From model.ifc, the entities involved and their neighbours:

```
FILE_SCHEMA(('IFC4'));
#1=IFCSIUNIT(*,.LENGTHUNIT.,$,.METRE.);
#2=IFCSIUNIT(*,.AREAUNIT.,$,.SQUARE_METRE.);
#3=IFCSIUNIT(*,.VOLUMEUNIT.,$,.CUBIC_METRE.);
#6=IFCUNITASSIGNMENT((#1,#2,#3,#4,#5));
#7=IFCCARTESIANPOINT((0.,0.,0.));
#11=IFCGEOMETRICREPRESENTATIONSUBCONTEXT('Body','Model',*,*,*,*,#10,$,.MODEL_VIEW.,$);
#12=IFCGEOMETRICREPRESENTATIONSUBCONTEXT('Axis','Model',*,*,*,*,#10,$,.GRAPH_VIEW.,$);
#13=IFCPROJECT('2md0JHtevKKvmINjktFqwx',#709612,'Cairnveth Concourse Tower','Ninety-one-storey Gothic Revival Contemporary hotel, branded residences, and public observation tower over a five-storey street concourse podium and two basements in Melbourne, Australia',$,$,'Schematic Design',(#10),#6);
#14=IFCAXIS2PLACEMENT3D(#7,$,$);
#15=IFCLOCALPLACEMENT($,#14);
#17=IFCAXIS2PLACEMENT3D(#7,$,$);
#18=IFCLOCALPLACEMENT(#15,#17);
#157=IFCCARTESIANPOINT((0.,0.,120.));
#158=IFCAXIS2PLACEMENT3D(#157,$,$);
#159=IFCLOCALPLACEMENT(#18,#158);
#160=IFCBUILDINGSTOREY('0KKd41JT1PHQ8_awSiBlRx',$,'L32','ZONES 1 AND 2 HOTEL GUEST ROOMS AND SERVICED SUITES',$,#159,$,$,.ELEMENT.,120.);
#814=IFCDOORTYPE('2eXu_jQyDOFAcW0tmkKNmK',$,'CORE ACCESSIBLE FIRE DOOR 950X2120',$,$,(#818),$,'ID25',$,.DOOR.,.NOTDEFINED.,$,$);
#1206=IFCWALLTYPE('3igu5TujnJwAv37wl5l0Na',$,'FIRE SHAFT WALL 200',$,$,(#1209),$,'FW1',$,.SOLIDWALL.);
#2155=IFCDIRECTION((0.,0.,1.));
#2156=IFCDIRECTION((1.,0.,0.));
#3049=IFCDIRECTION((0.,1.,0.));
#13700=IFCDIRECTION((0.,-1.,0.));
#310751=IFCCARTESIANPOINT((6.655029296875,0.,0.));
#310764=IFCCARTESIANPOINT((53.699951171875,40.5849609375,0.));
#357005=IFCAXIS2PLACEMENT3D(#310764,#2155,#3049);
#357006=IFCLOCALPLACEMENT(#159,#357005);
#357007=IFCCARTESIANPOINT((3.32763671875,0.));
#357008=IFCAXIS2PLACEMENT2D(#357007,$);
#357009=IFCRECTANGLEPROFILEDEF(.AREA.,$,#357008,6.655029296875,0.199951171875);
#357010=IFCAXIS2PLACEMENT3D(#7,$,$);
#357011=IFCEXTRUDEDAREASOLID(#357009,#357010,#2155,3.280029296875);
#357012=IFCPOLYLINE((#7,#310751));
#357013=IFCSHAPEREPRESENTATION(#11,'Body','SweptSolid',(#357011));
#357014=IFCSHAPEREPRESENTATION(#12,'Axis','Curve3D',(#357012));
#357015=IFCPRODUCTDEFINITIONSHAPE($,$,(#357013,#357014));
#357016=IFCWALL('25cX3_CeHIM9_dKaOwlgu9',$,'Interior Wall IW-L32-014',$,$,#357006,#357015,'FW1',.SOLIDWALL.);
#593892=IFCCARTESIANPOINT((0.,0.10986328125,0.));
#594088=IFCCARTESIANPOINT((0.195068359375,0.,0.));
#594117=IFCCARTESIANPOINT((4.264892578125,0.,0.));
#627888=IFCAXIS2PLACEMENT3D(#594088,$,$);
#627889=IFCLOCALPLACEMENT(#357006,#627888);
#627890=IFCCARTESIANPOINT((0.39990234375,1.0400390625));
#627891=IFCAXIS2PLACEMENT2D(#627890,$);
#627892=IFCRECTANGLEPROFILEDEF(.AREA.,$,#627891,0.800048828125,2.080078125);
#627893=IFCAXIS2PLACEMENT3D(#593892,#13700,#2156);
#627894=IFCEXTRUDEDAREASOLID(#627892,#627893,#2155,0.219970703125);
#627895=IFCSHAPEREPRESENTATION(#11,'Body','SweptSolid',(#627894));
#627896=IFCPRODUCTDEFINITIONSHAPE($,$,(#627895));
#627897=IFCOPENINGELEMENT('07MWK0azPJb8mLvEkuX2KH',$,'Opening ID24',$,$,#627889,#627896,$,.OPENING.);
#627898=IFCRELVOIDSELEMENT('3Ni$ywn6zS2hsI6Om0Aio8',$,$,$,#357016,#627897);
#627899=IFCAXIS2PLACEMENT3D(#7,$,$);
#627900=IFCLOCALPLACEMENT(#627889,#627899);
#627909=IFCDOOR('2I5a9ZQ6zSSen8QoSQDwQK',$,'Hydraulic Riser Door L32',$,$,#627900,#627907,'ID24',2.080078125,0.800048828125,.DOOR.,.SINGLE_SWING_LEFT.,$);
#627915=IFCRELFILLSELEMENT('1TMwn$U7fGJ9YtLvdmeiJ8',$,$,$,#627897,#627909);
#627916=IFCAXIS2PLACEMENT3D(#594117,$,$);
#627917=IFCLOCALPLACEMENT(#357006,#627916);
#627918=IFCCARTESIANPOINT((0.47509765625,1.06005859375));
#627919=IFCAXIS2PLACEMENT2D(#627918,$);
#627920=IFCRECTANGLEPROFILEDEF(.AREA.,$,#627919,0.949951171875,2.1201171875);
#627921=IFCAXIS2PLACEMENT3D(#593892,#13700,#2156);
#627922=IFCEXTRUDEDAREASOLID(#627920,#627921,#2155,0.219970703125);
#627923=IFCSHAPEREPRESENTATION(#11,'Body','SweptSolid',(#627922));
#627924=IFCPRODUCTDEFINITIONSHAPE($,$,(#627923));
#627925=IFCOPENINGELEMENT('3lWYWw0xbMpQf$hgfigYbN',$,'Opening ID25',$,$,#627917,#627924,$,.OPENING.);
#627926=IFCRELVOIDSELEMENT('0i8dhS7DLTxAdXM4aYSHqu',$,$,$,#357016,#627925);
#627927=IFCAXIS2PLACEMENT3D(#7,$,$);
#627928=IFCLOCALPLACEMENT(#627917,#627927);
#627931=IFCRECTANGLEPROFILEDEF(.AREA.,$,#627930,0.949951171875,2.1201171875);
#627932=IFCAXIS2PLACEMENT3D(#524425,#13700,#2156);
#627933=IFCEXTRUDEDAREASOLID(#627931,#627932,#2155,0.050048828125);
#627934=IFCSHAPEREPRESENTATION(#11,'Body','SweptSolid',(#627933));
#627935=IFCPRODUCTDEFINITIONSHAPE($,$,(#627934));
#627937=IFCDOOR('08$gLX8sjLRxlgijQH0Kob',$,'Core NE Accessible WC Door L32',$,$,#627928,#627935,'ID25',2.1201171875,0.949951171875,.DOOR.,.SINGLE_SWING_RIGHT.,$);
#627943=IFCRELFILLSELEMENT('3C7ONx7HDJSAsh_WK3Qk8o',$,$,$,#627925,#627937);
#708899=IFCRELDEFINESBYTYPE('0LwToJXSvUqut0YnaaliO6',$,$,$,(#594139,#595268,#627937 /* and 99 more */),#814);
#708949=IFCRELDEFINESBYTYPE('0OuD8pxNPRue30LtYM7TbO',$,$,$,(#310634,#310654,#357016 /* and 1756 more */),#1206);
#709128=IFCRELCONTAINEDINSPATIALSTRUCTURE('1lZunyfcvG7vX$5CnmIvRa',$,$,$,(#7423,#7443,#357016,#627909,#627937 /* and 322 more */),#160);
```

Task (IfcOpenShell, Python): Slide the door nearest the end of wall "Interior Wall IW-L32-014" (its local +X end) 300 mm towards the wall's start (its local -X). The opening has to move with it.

```python
import ifcopenshell
import ifcopenshell.api.geometry
import ifcopenshell.util.placement
import ifcopenshell.util.unit

model = ifcopenshell.open("model.ifc")
unit_scale = ifcopenshell.util.unit.calculate_unit_scale(model)

door = model.by_guid("08$gLX8sjLRxlgijQH0Kob")
opening = door.FillsVoids[0].RelatingOpeningElement
wall = opening.VoidsElements[0].RelatingBuildingElement

wall_matrix = ifcopenshell.util.placement.get_local_placement(wall.ObjectPlacement)
shift = wall_matrix[:3, 0] * -0.3 / unit_scale
before = ifcopenshell.util.placement.get_local_placement(door.ObjectPlacement)[:3, 3].copy()

# The door is placed relative to its opening, so it follows when the opening moves.
matrix = ifcopenshell.util.placement.get_local_placement(opening.ObjectPlacement)
matrix[:3, 3] += shift
ifcopenshell.api.geometry.edit_object_placement(
    model, product=opening, matrix=matrix, is_si=False, should_transform_children=True
)

after = ifcopenshell.util.placement.get_local_placement(door.ObjectPlacement)[:3, 3]
print("door moved by", (after - before).round(3) + 0.0)

model.write("model_edited.ifc")
```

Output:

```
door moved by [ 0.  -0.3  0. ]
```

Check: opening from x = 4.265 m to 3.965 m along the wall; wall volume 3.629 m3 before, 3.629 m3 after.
